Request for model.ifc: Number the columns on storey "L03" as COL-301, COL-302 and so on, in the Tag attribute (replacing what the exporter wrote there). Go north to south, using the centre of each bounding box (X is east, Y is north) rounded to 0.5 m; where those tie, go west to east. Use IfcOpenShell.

First a look at what the model holds.

```python
import ifcopenshell
import ifcopenshell.util.element
import ifcopenshell.util.placement

model = ifcopenshell.open("model.ifc")
print(model.schema)
storey = next(s for s in model.by_type("IfcBuildingStorey") if s.Name == "L03")
columns = [e for e in ifcopenshell.util.element.get_decomposition(storey) if e.is_a("IfcColumn")]
for e in sorted(columns, key=lambda e: e.id()):
    origin = ifcopenshell.util.placement.get_local_placement(e.ObjectPlacement)[:3, 3]
    print(e.id(), e.Tag, e.Name, origin.round(2) + 0.0, sep=" | ")
```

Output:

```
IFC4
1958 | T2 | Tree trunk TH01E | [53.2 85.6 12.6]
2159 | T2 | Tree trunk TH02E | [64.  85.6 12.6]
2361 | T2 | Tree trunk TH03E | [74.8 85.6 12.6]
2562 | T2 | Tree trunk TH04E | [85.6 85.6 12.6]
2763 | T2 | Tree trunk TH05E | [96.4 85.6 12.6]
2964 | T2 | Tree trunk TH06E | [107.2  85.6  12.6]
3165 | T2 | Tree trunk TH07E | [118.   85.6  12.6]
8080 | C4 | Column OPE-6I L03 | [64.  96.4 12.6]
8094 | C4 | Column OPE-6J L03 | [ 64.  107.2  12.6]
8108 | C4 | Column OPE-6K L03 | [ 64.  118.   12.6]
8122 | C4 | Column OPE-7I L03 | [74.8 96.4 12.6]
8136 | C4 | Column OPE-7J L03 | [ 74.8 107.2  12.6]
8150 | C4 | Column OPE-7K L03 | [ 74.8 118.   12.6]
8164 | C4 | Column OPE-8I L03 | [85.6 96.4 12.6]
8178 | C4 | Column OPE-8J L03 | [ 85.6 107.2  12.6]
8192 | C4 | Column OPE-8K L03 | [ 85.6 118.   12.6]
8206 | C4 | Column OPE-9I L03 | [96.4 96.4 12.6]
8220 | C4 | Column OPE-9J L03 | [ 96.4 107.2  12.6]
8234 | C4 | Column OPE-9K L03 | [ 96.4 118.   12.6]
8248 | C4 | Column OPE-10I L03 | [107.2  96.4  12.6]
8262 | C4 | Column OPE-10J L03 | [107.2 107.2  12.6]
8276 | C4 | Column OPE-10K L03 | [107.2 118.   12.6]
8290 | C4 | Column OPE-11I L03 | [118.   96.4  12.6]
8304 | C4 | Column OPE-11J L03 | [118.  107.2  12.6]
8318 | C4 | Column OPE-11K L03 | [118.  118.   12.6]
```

```python
import ifcopenshell
import ifcopenshell.geom
import ifcopenshell.util.element
import ifcopenshell.util.shape

model = ifcopenshell.open("model.ifc")
settings = ifcopenshell.geom.settings()
settings.set("use-world-coords", True)


def centre(element):
    shape = ifcopenshell.geom.create_shape(settings, element)
    return ifcopenshell.util.shape.get_bbox_centroid(shape.geometry)


storey = next(s for s in model.by_type("IfcBuildingStorey") if s.Name == "L03")
columns = [e for e in ifcopenshell.util.element.get_decomposition(storey) if e.is_a("IfcColumn")]

# Insertion points can sit at a corner or the storey origin, so sort by the geometry (in metres).
centres = {e: centre(e) for e in columns}
columns.sort(key=lambda e: (-round(centres[e][1] / 0.5), centres[e][0]))

for i, e in enumerate(columns, start=1):
    number = f"COL-3{i:02d}"
    e.Tag = number
    print(e.id(), number)

model.write("model_edited.ifc")
```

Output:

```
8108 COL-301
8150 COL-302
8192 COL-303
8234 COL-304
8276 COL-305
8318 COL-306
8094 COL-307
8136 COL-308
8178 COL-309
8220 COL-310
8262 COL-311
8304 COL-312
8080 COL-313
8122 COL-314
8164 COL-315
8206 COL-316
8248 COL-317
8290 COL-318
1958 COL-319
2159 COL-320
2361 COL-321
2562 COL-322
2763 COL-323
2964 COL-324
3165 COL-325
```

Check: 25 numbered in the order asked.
